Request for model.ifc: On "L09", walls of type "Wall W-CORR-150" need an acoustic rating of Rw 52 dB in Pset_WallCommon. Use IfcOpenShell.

First a look at what the model holds.

```python
import ifcopenshell
import ifcopenshell.util.element

model = ifcopenshell.open("model.ifc")
print(model.schema)
storey = next(s for s in model.by_type("IfcBuildingStorey") if s.Name == "L09")
walls = [e for e in ifcopenshell.util.element.get_decomposition(storey) if e.is_a("IfcWall")]
seen = {}
for e in walls:
    element_type = ifcopenshell.util.element.get_type(e)
    key = (element_type.Name if element_type != e and element_type else None, ifcopenshell.util.element.get_pset(e, "Pset_WallCommon", "AcousticRating"))
    seen[key] = seen.get(key, 0) + 1
for (name, value), count in sorted(seen.items(), key=str):
    print(count, "x", name, "|", value)
```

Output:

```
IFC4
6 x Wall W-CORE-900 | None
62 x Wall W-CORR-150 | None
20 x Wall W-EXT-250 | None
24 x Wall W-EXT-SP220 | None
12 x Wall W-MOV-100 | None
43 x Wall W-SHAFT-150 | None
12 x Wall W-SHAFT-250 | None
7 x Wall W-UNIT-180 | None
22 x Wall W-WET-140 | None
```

```python
import ifcopenshell
import ifcopenshell.api.pset
import ifcopenshell.util.element

model = ifcopenshell.open("model.ifc")

storey = next(s for s in model.by_type("IfcBuildingStorey") if s.Name == "L09")
walls = [e for e in ifcopenshell.util.element.get_decomposition(storey) if e.is_a("IfcWall")]

count = 0
for e in walls:
    element_type = ifcopenshell.util.element.get_type(e)
    if element_type in (None, e) or element_type.Name != "Wall W-CORR-150":
        continue
    found = ifcopenshell.util.element.get_pset(e, "Pset_WallCommon", should_inherit=False)
    if found:
        pset = model.by_id(found["id"])
        if len(ifcopenshell.util.element.get_elements_by_pset(pset)) > 1:
            pset = ifcopenshell.api.pset.unshare_pset(model, products=[e], pset=pset)[0]
    else:
        pset = ifcopenshell.api.pset.add_pset(model, product=e, name="Pset_WallCommon")
    ifcopenshell.api.pset.edit_pset(model, pset=pset, properties={"AcousticRating": "Rw 52 dB"})
    count += 1

print(count, "walls updated")

model.write("model_v2.ifc")
```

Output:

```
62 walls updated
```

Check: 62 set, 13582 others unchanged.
